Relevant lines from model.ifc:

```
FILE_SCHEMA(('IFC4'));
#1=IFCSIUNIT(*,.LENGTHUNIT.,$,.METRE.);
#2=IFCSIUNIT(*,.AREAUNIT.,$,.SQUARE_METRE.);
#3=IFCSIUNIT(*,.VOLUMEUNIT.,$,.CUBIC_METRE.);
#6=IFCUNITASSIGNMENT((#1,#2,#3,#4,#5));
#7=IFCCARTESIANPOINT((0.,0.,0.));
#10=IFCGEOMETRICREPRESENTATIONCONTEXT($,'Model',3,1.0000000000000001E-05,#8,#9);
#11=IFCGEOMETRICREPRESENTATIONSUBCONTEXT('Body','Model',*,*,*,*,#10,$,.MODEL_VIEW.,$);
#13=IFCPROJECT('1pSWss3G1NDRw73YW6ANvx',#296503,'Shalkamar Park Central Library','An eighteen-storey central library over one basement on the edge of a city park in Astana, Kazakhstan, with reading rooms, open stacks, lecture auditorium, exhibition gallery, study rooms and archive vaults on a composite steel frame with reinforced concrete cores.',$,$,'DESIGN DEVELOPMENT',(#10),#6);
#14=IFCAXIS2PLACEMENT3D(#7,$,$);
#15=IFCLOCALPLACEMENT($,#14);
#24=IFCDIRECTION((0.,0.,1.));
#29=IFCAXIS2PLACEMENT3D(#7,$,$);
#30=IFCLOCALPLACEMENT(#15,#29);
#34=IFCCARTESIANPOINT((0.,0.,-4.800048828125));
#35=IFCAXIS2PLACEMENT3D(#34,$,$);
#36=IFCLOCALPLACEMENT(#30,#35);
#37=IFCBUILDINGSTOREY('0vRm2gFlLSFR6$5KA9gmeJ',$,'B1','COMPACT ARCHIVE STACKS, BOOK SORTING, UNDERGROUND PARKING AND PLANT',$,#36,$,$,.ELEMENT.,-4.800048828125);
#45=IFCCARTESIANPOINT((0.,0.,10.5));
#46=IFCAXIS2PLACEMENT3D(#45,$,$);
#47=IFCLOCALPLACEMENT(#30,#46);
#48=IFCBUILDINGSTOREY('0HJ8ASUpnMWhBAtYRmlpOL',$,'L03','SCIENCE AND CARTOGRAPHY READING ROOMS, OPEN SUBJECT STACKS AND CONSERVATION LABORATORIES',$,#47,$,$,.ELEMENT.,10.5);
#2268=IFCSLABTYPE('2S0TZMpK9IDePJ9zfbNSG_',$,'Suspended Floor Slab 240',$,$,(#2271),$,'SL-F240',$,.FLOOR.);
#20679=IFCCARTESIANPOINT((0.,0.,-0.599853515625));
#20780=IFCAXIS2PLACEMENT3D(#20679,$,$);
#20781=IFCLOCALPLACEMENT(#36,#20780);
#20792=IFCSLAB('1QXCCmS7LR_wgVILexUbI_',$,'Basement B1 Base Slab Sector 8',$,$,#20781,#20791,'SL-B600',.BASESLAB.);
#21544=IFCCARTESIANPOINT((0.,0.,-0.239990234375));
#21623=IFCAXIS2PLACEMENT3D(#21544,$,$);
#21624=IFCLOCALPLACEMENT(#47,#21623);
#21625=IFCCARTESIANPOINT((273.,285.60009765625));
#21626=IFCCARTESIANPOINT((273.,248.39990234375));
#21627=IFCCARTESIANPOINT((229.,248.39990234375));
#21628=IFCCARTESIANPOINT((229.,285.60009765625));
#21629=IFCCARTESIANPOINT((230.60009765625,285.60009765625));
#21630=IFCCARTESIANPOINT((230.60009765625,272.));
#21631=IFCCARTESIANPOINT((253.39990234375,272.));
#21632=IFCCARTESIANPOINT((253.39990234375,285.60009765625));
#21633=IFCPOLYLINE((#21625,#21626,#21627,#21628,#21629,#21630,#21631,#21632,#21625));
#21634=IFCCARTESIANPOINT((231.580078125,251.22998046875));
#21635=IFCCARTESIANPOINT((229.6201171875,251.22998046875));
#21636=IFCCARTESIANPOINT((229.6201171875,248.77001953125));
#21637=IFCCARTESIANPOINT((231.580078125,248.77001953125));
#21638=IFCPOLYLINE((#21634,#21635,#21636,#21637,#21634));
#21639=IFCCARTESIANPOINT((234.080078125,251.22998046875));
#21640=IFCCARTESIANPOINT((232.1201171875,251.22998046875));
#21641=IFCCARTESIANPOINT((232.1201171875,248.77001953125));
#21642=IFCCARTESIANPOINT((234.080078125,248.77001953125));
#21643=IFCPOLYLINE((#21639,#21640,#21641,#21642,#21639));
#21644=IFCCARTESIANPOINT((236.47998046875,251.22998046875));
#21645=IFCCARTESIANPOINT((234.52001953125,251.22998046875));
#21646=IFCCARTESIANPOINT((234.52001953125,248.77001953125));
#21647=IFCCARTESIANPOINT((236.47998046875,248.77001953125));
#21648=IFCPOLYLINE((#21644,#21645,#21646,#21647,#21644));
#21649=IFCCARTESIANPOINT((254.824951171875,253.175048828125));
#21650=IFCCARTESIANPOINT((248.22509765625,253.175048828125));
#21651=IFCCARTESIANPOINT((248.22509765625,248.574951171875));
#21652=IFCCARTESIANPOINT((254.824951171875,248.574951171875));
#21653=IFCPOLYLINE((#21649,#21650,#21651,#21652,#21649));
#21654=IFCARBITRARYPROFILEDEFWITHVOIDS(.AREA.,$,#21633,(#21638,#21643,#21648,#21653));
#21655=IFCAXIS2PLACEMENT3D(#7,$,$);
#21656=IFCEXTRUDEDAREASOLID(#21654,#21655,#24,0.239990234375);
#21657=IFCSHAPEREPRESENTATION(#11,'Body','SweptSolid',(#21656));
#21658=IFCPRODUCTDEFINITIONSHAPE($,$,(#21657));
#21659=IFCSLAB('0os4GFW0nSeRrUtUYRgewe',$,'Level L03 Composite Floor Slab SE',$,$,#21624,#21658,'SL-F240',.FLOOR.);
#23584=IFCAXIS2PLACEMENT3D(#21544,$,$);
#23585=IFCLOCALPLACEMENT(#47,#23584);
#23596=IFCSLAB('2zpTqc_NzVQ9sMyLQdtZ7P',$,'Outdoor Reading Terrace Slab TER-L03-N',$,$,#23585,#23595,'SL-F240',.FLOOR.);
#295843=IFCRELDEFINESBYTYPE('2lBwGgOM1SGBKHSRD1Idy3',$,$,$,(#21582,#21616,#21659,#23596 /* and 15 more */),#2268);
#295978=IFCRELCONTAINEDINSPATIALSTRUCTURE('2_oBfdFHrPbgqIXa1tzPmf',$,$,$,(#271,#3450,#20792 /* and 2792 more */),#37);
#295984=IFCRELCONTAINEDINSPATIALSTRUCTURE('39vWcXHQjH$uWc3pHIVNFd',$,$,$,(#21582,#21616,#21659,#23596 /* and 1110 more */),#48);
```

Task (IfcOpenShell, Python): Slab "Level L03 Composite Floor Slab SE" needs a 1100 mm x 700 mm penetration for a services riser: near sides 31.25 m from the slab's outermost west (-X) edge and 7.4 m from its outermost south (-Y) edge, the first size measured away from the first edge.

```python
import numpy as np
import ifcopenshell
import ifcopenshell.api.feature
import ifcopenshell.api.geometry
import ifcopenshell.api.root
import ifcopenshell.geom
import ifcopenshell.util.placement
import ifcopenshell.util.representation
import ifcopenshell.util.shape
import ifcopenshell.util.unit

model = ifcopenshell.open("model.ifc")
unit_scale = ifcopenshell.util.unit.calculate_unit_scale(model)
settings = ifcopenshell.geom.settings()


def volume(element):
    """Net volume in cubic metres, openings subtracted."""
    shape = ifcopenshell.geom.create_shape(settings, element)
    return ifcopenshell.util.shape.get_volume(shape.geometry)


slab = model.by_guid("0os4GFW0nSeRrUtUYRgewe")
before = volume(slab)

# Extent in the slab's own axes, in metres. The edges named are its -X and -Y sides.
slab_shape = ifcopenshell.geom.create_shape(settings, slab)
vertices = ifcopenshell.util.shape.get_vertices(slab_shape.geometry)
x_min, y_min, bottom = vertices.min(axis=0)
top = vertices[:, 2].max()

opening = ifcopenshell.api.root.create_entity(model, ifc_class="IfcOpeningElement", name="Services riser opening", predefined_type="OPENING")
context = ifcopenshell.util.representation.get_context(model, "Model", "Body", "MODEL_VIEW")
width, depth = 1.1, 0.7
outline = [(0.0, 0.0), (width, 0.0), (width, depth), (0.0, depth), (0.0, 0.0)]
# Overshoot both faces by 50 mm so the cut is clean.
shape = ifcopenshell.api.geometry.add_slab_representation(
    model, context=context, depth=top - bottom + 0.1, polyline=outline
)
ifcopenshell.api.geometry.assign_representation(model, product=opening, representation=shape)

matrix = ifcopenshell.util.placement.get_local_placement(slab.ObjectPlacement)
matrix[:, 3] = matrix @ np.append(np.array([x_min + 31.25, y_min + 7.4, bottom - 0.05]) / unit_scale, 1.0)
ifcopenshell.api.geometry.edit_object_placement(model, product=opening, matrix=matrix, is_si=False)
ifcopenshell.api.feature.add_feature(model, feature=opening, element=slab)

after = volume(slab)

print(f"slab volume {before:.3f} -> {after:.3f} m3")

model.write("model-out.ifc")
```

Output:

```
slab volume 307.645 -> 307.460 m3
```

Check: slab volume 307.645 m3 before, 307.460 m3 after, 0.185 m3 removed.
